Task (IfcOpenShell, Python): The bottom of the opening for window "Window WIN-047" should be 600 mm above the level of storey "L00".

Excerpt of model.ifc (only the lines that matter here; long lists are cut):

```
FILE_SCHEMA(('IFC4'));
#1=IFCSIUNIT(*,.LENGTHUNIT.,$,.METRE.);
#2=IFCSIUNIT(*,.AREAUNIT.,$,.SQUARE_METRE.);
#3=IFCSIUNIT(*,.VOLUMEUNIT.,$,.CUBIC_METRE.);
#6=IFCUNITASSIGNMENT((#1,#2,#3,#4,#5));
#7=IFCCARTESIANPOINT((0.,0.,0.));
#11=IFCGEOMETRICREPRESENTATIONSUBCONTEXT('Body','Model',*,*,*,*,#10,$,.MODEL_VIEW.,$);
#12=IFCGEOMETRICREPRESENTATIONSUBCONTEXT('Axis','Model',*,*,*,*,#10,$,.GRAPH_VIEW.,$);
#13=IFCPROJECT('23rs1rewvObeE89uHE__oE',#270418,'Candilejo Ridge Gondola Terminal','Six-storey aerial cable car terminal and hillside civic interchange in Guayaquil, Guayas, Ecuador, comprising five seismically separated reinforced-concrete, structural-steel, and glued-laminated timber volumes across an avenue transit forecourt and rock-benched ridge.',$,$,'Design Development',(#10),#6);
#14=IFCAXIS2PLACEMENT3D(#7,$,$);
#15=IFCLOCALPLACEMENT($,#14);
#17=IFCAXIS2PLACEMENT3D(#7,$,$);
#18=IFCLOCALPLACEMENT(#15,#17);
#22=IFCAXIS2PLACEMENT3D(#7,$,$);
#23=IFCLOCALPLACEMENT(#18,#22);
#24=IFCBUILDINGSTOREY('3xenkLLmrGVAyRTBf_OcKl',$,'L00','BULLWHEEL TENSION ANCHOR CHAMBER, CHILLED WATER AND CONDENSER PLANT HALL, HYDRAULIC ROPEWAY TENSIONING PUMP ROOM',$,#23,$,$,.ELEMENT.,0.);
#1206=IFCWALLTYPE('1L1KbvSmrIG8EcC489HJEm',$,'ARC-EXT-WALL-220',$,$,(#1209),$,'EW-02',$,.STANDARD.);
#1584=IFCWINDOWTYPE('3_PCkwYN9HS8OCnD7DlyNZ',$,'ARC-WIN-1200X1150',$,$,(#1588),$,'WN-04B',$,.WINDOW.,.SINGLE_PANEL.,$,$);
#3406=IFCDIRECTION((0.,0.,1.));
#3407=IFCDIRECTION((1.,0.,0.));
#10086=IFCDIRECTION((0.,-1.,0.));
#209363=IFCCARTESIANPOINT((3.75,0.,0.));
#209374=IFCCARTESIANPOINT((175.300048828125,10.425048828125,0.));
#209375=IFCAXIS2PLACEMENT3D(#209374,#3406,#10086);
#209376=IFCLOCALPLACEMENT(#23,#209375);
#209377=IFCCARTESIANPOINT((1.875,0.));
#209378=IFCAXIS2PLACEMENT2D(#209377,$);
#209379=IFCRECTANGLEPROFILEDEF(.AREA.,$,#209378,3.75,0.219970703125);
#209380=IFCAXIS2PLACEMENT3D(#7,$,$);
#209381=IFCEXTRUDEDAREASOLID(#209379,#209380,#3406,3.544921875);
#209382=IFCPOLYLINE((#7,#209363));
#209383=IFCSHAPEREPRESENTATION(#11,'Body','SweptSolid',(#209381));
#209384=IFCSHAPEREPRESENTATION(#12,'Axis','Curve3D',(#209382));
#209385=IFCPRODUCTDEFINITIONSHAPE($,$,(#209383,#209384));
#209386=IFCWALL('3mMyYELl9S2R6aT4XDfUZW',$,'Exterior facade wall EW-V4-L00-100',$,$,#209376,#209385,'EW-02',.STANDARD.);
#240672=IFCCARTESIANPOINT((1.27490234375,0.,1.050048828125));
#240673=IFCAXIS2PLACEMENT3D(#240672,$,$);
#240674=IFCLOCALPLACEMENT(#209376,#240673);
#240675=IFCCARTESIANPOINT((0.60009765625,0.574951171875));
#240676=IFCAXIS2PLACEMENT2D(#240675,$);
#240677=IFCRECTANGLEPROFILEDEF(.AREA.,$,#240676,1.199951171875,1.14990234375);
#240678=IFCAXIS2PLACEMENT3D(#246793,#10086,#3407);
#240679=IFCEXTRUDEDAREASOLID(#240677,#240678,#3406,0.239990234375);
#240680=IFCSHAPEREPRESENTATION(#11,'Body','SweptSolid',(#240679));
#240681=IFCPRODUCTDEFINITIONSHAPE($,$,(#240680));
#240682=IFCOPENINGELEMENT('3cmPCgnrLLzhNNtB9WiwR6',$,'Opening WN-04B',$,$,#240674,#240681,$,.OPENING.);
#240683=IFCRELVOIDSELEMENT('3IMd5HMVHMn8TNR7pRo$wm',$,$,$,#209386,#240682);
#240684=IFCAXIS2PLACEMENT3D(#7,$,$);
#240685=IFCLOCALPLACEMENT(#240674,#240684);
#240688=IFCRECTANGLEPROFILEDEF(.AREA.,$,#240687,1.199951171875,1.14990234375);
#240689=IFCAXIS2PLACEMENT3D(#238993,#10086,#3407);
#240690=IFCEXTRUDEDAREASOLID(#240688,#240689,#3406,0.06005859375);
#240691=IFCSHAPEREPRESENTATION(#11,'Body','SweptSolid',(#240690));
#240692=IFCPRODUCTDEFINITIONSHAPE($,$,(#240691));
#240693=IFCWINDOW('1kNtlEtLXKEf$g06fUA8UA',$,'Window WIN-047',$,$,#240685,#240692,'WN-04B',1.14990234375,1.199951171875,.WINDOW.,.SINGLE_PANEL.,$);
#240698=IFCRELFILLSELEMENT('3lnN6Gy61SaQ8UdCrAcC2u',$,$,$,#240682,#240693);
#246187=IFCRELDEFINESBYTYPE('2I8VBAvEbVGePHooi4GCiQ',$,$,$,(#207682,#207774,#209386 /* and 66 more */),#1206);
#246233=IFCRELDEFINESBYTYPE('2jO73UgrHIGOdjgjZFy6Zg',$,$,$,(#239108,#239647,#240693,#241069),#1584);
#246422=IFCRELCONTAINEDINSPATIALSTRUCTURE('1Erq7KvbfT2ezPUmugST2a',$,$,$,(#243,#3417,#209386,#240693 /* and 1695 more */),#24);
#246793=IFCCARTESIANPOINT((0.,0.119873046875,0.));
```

```python
import numpy as np
import ifcopenshell
import ifcopenshell.api.geometry
import ifcopenshell.geom
import ifcopenshell.util.element
import ifcopenshell.util.placement
import ifcopenshell.util.shape
import ifcopenshell.util.unit

model = ifcopenshell.open("model.ifc")
unit_scale = ifcopenshell.util.unit.calculate_unit_scale(model)

window = model.by_id(240693)
opening = window.FillsVoids[0].RelatingOpeningElement
storey = ifcopenshell.util.element.get_container(window, ifc_class="IfcBuildingStorey")
level = ifcopenshell.util.placement.get_local_placement(storey.ObjectPlacement)[2, 3]

# The opening's origin need not be at the sill, so measure its lowest point.
shape = ifcopenshell.geom.create_shape(ifcopenshell.geom.settings(), opening)
bottom = ifcopenshell.util.shape.get_shape_bottom_elevation(shape, shape.geometry) / unit_scale
dz = level + 0.6 / unit_scale - bottom

shift = np.array([0.0, 0.0, dz])
# The window is placed relative to its opening, so it follows when the opening moves.
matrix = ifcopenshell.util.placement.get_local_placement(opening.ObjectPlacement)
matrix[:3, 3] += shift
ifcopenshell.api.geometry.edit_object_placement(
    model, product=opening, matrix=matrix, is_si=False, should_transform_children=True
)

print(f"moved by {dz * unit_scale:+.3f} m")

model.write("model_updated.ifc")
```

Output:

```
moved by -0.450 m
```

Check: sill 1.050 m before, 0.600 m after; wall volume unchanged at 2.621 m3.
